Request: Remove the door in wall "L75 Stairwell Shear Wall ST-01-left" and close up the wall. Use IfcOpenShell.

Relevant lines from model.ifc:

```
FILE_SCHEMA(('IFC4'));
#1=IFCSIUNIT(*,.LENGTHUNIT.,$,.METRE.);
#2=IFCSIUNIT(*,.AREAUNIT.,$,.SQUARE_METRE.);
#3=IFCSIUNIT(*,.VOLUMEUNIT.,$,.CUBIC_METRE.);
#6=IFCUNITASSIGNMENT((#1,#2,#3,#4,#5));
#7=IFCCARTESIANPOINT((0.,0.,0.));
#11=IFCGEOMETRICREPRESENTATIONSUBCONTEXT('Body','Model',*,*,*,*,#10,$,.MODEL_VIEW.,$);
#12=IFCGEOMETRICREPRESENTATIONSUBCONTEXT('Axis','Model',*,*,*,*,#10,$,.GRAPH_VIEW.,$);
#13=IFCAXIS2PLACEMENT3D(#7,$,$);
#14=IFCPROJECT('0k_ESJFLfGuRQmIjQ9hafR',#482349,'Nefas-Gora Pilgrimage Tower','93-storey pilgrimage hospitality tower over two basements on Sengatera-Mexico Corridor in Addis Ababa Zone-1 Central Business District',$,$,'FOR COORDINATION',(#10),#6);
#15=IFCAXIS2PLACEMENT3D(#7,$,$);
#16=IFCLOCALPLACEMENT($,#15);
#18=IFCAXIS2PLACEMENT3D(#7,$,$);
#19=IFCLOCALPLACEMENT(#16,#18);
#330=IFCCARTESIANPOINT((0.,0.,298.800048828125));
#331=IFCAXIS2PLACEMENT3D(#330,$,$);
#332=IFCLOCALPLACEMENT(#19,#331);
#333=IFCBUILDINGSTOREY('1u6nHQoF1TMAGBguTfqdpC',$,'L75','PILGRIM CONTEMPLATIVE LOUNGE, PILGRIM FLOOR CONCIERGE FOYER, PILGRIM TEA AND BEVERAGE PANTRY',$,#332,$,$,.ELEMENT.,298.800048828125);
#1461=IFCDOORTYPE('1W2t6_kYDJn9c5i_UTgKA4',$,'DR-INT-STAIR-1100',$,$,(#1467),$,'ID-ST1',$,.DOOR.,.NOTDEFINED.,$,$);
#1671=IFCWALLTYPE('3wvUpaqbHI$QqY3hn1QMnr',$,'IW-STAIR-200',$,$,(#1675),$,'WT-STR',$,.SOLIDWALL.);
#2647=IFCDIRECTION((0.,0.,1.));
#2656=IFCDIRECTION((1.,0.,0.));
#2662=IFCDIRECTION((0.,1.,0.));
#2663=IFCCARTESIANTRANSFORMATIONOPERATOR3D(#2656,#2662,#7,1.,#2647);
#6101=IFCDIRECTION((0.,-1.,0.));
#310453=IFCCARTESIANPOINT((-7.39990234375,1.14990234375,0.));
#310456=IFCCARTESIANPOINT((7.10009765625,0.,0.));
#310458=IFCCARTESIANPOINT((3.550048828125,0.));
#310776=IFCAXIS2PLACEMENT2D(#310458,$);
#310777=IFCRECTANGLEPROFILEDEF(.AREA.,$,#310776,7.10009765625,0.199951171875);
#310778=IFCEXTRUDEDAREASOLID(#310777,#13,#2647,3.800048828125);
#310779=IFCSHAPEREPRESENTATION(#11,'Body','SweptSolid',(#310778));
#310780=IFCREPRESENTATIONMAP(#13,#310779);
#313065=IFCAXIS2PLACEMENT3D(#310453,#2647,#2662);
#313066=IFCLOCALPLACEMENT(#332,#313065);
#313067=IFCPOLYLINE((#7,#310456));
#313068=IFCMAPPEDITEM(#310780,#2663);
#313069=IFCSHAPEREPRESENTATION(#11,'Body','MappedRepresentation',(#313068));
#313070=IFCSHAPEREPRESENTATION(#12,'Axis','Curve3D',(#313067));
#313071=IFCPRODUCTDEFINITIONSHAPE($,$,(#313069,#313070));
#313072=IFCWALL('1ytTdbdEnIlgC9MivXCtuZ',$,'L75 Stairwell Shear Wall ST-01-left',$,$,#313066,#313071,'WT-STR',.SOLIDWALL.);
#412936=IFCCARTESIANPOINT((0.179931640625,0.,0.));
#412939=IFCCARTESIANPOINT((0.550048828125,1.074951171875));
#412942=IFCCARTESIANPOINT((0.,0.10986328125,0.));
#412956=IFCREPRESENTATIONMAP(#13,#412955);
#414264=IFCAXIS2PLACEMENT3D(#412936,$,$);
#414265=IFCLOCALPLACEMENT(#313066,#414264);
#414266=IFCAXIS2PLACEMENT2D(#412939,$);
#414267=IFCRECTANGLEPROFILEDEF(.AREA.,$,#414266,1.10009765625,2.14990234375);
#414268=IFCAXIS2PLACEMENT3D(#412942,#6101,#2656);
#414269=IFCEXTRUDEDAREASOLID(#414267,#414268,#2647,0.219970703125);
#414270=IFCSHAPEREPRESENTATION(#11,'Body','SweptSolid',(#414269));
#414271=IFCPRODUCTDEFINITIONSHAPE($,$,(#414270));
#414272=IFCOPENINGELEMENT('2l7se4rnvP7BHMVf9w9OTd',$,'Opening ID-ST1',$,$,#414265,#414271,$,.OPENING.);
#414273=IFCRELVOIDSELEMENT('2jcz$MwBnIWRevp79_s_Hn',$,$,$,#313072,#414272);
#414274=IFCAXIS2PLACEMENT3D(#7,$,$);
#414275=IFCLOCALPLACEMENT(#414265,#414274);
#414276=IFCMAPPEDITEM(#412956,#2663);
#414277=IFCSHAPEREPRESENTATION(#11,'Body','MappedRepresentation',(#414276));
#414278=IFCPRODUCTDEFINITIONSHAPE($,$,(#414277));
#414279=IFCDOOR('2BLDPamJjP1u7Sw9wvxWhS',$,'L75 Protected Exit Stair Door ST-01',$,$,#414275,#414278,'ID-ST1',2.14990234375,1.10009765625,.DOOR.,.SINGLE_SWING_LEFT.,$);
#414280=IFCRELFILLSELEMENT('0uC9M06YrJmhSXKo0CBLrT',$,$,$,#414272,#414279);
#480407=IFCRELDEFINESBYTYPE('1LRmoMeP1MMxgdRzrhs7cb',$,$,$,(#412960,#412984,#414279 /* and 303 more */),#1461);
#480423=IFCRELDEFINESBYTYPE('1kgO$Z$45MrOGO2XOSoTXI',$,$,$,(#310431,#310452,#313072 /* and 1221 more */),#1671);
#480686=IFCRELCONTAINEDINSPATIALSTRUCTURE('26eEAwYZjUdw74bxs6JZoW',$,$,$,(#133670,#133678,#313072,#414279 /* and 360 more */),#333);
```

```python
import ifcopenshell
import ifcopenshell.api.feature
import ifcopenshell.api.root
import ifcopenshell.geom
import ifcopenshell.util.shape

model = ifcopenshell.open("model.ifc")
settings = ifcopenshell.geom.settings()


def volume(element):
    """Net volume in cubic metres, openings subtracted."""
    shape = ifcopenshell.geom.create_shape(settings, element)
    return ifcopenshell.util.shape.get_volume(shape.geometry)


door = model.by_guid("2BLDPamJjP1u7Sw9wvxWhS")
opening = door.FillsVoids[0].RelatingOpeningElement
wall = opening.VoidsElements[0].RelatingBuildingElement
before = volume(wall)

ifcopenshell.api.root.remove_product(model, product=door)
ifcopenshell.api.feature.remove_feature(model, feature=opening)

after = volume(wall)

print(f"wall volume {before:.3f} -> {after:.3f} m3")

model.write("model-out.ifc")
```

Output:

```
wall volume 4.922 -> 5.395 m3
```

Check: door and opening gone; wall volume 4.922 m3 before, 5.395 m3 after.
